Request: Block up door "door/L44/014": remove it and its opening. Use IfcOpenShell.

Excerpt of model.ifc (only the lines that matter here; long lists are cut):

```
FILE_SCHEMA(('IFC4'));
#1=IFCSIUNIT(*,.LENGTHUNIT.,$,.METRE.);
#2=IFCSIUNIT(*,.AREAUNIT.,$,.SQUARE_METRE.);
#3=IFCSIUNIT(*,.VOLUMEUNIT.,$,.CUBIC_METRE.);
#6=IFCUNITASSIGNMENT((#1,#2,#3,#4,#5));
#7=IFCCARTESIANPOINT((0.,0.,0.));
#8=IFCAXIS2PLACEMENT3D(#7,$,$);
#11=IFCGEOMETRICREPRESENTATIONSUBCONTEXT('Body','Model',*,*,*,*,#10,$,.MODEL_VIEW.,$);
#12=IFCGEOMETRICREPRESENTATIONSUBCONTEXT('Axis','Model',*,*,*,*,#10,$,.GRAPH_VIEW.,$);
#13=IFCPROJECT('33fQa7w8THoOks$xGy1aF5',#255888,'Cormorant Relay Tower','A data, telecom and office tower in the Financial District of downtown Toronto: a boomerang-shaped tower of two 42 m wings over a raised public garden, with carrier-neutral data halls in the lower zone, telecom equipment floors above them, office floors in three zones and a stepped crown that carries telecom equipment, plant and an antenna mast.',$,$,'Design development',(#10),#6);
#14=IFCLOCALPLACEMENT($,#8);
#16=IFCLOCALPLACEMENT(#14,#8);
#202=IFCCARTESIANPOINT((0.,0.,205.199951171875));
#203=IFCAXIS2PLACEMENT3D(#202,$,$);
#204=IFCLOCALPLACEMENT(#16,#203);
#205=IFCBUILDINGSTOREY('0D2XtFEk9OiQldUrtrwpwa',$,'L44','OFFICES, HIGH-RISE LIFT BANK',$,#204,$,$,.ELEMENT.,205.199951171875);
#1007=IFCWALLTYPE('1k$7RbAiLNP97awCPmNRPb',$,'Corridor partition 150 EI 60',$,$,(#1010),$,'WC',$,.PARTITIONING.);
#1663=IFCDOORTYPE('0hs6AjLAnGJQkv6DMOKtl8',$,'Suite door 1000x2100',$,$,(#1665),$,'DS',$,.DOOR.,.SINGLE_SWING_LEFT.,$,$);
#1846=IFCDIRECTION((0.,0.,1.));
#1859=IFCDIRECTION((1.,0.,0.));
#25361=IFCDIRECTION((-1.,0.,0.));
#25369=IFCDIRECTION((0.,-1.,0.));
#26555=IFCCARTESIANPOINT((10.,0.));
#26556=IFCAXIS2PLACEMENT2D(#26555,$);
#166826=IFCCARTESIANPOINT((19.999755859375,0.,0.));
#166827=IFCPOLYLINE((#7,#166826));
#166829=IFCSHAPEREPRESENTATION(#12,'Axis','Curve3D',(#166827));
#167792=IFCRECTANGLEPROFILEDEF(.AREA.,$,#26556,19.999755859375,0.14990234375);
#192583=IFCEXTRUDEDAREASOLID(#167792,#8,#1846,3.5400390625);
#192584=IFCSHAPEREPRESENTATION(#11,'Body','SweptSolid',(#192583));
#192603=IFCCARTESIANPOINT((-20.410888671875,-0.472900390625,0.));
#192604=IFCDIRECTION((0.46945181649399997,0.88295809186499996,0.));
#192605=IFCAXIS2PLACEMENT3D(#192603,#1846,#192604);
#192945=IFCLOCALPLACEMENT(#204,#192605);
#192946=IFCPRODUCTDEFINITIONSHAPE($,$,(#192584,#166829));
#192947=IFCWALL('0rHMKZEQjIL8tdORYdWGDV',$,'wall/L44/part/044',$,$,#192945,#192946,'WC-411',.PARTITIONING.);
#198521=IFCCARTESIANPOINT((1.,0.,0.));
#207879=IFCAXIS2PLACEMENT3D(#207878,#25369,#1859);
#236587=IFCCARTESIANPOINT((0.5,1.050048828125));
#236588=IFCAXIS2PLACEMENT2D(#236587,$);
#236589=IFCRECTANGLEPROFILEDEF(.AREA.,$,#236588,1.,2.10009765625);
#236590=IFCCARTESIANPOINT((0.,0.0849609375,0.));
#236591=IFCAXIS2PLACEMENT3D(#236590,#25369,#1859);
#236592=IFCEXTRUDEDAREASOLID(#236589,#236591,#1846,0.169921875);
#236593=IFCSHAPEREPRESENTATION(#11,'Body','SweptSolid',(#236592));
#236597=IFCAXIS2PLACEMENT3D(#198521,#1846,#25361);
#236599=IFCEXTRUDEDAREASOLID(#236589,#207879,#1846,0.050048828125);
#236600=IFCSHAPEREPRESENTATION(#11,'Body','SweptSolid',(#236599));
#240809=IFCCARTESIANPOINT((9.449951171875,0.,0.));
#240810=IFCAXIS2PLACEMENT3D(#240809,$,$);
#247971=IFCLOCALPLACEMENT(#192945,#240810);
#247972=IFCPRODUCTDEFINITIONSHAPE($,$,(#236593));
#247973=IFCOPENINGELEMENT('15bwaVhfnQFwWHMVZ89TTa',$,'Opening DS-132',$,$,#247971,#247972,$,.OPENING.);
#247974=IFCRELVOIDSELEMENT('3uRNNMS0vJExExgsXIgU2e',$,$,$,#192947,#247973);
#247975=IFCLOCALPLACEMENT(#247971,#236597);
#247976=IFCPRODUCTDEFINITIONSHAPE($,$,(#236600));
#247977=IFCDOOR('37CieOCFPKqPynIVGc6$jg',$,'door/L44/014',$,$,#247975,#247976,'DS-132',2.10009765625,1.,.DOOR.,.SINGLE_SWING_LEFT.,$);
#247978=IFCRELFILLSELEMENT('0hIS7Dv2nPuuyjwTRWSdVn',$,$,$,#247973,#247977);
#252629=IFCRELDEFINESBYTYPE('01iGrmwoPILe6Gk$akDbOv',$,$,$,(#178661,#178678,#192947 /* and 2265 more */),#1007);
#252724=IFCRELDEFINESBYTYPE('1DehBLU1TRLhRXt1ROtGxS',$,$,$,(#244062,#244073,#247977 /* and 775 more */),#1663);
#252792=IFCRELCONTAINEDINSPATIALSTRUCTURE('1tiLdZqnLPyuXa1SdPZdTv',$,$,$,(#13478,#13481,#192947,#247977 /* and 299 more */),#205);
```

```python
import ifcopenshell
import ifcopenshell.api.feature
import ifcopenshell.api.root
import ifcopenshell.geom
import ifcopenshell.util.shape

model = ifcopenshell.open("model.ifc")
settings = ifcopenshell.geom.settings()


def volume(element):
    """Net volume in cubic metres, openings subtracted."""
    shape = ifcopenshell.geom.create_shape(settings, element)
    return ifcopenshell.util.shape.get_volume(shape.geometry)


door = model.by_id(247977)
opening = door.FillsVoids[0].RelatingOpeningElement
wall = opening.VoidsElements[0].RelatingBuildingElement
before = volume(wall)

ifcopenshell.api.root.remove_product(model, product=door)
ifcopenshell.api.feature.remove_feature(model, feature=opening)

after = volume(wall)

print(f"wall volume {before:.3f} -> {after:.3f} m3")

model.write("model-out.ifc")
```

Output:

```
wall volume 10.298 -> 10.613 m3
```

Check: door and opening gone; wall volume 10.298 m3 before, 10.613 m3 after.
